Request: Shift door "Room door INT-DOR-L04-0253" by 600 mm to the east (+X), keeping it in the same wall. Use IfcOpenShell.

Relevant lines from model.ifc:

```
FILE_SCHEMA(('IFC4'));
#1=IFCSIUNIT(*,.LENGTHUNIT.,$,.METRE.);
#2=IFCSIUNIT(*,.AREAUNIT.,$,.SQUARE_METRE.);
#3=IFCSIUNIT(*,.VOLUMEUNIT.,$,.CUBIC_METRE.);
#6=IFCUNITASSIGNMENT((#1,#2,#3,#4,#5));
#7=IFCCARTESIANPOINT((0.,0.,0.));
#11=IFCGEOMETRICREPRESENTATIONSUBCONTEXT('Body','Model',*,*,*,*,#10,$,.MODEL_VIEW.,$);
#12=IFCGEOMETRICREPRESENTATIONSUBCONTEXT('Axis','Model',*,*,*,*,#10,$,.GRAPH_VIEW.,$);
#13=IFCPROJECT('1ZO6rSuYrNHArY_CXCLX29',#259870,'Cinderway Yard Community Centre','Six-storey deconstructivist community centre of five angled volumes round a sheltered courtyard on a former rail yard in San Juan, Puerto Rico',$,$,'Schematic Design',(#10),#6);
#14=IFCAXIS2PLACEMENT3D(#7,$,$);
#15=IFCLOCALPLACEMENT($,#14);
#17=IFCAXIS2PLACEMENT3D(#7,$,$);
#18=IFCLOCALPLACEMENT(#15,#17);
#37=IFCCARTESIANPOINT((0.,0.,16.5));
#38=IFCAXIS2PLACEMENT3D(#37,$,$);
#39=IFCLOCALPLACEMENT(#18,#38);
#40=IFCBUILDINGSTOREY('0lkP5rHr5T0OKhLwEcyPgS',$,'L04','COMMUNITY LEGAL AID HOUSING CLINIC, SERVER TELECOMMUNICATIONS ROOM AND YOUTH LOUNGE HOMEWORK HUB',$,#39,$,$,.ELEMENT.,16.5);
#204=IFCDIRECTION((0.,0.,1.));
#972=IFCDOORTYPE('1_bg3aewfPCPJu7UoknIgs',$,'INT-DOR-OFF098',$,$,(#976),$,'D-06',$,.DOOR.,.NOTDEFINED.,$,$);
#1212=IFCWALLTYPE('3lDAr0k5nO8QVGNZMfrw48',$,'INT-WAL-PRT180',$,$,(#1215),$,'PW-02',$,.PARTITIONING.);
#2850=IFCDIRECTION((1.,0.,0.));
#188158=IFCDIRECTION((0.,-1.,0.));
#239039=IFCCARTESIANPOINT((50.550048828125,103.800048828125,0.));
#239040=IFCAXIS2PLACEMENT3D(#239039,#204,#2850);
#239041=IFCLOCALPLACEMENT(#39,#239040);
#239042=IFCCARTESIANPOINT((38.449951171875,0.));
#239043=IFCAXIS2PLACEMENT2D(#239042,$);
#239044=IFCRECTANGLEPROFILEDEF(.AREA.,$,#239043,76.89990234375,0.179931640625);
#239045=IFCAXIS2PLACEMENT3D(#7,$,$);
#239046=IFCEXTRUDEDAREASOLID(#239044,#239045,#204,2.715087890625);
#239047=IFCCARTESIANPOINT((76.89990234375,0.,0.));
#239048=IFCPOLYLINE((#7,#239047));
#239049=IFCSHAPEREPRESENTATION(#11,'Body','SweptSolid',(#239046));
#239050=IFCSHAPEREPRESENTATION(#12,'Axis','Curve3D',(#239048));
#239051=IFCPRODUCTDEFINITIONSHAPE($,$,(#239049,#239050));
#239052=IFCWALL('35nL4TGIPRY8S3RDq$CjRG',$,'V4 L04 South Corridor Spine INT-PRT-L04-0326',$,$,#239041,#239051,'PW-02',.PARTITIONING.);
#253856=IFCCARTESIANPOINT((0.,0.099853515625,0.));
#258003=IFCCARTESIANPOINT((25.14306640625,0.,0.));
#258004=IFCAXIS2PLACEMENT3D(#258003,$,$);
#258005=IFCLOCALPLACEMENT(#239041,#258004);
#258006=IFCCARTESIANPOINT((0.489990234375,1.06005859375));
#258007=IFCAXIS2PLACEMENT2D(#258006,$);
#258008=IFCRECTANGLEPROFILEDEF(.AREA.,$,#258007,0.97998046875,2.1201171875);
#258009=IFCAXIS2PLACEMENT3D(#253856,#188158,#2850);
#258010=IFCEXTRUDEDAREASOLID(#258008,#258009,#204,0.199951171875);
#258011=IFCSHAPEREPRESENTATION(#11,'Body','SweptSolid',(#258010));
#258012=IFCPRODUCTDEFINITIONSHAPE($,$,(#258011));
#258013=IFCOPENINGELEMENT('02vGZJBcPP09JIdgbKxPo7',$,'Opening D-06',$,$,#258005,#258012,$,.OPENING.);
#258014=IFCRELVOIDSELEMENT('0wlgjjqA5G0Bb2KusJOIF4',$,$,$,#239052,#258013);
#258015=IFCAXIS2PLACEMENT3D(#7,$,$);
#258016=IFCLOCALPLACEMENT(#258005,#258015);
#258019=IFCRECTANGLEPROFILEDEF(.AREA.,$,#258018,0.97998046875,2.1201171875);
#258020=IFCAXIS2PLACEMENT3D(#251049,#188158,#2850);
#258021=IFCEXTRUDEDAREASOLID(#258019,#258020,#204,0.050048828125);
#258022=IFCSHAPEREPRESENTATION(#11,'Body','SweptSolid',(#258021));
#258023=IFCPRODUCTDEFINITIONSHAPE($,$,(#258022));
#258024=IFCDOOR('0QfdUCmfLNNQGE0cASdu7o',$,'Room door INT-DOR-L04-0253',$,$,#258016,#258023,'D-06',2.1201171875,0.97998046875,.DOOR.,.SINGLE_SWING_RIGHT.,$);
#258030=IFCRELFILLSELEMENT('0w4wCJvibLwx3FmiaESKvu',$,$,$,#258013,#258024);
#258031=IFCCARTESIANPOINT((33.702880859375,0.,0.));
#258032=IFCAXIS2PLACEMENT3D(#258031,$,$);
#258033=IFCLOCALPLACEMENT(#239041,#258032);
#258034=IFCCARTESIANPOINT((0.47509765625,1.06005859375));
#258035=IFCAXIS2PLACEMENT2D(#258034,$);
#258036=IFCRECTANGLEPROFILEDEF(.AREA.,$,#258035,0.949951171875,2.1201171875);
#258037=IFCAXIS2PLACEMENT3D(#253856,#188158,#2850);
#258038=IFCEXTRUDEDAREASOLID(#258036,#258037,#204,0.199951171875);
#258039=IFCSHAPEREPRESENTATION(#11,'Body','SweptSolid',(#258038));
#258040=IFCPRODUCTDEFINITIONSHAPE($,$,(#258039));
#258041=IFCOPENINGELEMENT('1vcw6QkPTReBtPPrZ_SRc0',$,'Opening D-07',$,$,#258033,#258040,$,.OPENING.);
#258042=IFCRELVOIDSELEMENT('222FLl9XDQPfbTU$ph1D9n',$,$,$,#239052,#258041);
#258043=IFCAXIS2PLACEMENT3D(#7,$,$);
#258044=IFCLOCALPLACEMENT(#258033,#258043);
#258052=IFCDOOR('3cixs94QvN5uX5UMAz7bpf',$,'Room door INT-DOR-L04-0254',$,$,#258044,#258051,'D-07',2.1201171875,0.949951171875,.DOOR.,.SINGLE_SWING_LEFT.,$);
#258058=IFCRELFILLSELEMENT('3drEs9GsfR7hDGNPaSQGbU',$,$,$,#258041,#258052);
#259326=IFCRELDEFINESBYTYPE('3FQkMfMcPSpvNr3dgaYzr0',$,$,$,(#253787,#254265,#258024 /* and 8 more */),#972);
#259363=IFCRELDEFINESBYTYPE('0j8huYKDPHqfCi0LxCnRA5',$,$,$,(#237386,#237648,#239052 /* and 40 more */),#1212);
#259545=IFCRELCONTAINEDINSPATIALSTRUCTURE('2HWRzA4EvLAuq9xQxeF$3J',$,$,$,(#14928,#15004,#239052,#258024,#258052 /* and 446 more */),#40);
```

```python
import ifcopenshell
import ifcopenshell.api.geometry
import ifcopenshell.util.placement

model = ifcopenshell.open("model.ifc")

door = model.by_id(258024)
opening = door.FillsVoids[0].RelatingOpeningElement
wall = opening.VoidsElements[0].RelatingBuildingElement

wall_matrix = ifcopenshell.util.placement.get_local_placement(wall.ObjectPlacement)
shift = wall_matrix[:3, 0] * 0.6
before = ifcopenshell.util.placement.get_local_placement(door.ObjectPlacement)[:3, 3].copy()

# The door is placed relative to its opening, so it follows when the opening moves.
matrix = ifcopenshell.util.placement.get_local_placement(opening.ObjectPlacement)
matrix[:3, 3] += shift
ifcopenshell.api.geometry.edit_object_placement(
    model, product=opening, matrix=matrix, is_si=False, should_transform_children=True
)

after = ifcopenshell.util.placement.get_local_placement(door.ObjectPlacement)[:3, 3]
print("door moved by", (after - before).round(3) + 0.0)

model.write("model-out.ifc")
```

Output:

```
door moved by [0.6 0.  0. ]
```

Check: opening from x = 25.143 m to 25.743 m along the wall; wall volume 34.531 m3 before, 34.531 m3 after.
